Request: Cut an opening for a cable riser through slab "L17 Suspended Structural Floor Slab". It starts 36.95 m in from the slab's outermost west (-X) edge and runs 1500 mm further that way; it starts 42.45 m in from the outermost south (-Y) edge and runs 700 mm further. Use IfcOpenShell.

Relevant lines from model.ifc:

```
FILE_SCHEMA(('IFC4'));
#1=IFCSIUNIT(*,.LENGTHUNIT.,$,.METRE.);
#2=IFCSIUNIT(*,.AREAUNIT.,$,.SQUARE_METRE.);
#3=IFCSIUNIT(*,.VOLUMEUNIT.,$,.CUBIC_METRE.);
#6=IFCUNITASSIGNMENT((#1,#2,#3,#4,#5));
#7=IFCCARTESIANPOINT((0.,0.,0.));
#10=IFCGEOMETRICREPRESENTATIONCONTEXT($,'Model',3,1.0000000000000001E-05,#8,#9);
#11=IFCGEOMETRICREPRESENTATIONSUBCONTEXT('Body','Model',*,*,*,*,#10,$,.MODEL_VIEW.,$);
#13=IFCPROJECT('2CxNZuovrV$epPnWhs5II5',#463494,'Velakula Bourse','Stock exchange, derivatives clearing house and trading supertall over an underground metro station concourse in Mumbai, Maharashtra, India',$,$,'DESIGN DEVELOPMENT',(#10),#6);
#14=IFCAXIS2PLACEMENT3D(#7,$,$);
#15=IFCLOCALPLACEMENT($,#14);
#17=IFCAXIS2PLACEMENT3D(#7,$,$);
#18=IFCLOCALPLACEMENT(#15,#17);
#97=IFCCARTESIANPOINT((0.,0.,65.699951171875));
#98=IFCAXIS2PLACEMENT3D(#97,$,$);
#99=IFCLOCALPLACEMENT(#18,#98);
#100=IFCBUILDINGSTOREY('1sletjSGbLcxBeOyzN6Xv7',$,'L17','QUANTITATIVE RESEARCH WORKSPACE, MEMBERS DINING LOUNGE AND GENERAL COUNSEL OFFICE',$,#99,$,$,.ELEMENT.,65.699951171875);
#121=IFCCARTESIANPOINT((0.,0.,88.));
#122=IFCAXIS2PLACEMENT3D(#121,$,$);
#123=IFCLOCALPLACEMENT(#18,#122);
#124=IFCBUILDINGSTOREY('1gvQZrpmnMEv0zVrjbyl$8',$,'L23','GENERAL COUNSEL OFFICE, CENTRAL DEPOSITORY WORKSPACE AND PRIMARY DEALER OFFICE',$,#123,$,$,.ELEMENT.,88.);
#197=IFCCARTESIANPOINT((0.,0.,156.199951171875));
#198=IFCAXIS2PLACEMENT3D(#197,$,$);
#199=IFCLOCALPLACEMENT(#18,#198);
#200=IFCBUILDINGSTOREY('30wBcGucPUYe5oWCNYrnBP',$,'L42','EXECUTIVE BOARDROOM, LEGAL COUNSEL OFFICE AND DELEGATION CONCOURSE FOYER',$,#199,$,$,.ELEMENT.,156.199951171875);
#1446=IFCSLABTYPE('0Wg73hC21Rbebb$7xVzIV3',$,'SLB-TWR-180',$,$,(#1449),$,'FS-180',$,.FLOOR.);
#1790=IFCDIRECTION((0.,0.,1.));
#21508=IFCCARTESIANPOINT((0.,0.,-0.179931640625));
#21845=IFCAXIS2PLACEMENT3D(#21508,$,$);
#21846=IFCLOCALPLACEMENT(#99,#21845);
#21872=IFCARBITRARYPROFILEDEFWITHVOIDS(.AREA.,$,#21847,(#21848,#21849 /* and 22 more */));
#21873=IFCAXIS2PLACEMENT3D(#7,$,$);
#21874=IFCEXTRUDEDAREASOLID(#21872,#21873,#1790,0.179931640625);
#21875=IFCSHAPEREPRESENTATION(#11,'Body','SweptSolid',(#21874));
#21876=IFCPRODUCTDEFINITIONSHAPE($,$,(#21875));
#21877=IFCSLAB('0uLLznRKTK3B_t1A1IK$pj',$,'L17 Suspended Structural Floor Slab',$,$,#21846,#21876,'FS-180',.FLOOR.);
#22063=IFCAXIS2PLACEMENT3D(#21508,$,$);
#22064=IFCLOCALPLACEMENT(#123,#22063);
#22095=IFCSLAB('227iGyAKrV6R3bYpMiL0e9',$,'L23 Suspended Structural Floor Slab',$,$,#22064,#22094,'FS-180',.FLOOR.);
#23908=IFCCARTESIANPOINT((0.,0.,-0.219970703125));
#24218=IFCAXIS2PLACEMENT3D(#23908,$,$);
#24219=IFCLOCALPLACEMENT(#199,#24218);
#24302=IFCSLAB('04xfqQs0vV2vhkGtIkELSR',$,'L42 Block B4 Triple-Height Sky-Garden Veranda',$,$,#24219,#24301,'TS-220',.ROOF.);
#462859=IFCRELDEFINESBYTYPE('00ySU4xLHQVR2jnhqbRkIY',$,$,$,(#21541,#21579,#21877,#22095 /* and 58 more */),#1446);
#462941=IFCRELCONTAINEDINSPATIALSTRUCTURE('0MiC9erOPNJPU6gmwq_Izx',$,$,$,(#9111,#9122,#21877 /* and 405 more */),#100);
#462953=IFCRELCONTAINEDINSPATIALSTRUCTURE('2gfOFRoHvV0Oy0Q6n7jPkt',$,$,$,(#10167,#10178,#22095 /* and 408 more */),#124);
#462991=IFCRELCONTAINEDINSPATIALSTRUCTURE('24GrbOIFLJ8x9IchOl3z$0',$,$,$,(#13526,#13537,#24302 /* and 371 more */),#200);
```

```python
import numpy as np
import ifcopenshell
import ifcopenshell.api.feature
import ifcopenshell.api.geometry
import ifcopenshell.api.root
import ifcopenshell.geom
import ifcopenshell.util.placement
import ifcopenshell.util.representation
import ifcopenshell.util.shape
import ifcopenshell.util.unit

model = ifcopenshell.open("model.ifc")
unit_scale = ifcopenshell.util.unit.calculate_unit_scale(model)
settings = ifcopenshell.geom.settings()


def volume(element):
    """Net volume in cubic metres, openings subtracted."""
    shape = ifcopenshell.geom.create_shape(settings, element)
    return ifcopenshell.util.shape.get_volume(shape.geometry)


slab = model.by_id(21877)
before = volume(slab)

# Extent in the slab's own axes, in metres. The edges named are its -X and -Y sides.
slab_shape = ifcopenshell.geom.create_shape(settings, slab)
vertices = ifcopenshell.util.shape.get_vertices(slab_shape.geometry)
x_min, y_min, bottom = vertices.min(axis=0)
top = vertices[:, 2].max()

opening = ifcopenshell.api.root.create_entity(model, ifc_class="IfcOpeningElement", name="Cable riser opening", predefined_type="OPENING")
context = ifcopenshell.util.representation.get_context(model, "Model", "Body", "MODEL_VIEW")
width, depth = 1.5, 0.7
outline = [(0.0, 0.0), (width, 0.0), (width, depth), (0.0, depth), (0.0, 0.0)]
# Overshoot both faces by 50 mm so the cut is clean.
shape = ifcopenshell.api.geometry.add_slab_representation(
    model, context=context, depth=top - bottom + 0.1, polyline=outline
)
ifcopenshell.api.geometry.assign_representation(model, product=opening, representation=shape)

matrix = ifcopenshell.util.placement.get_local_placement(slab.ObjectPlacement)
matrix[:, 3] = matrix @ np.append(np.array([x_min + 36.95, y_min + 42.45, bottom - 0.05]) / unit_scale, 1.0)
ifcopenshell.api.geometry.edit_object_placement(model, product=opening, matrix=matrix, is_si=False)
ifcopenshell.api.feature.add_feature(model, feature=opening, element=slab)

after = volume(slab)

print(f"slab volume {before:.3f} -> {after:.3f} m3")

model.write("model_updated.ifc")
```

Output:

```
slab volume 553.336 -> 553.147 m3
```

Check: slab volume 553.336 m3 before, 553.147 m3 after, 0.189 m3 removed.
